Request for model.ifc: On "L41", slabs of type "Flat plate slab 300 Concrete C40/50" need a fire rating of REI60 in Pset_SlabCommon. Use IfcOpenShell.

First a look at what the model holds.

```python
import ifcopenshell
import ifcopenshell.util.element

model = ifcopenshell.open("model.ifc")
print(model.schema)
storey = next(s for s in model.by_type("IfcBuildingStorey") if s.Name == "L41")
slabs = [e for e in ifcopenshell.util.element.get_decomposition(storey) if e.is_a("IfcSlab")]
seen = {}
for e in slabs:
    element_type = ifcopenshell.util.element.get_type(e)
    key = (element_type.Name if element_type != e and element_type else None, ifcopenshell.util.element.get_pset(e, "Pset_SlabCommon", "FireRating"))
    seen[key] = seen.get(key, 0) + 1
for (name, value), count in sorted(seen.items(), key=str):
    print(count, "x", name, "|", value)
```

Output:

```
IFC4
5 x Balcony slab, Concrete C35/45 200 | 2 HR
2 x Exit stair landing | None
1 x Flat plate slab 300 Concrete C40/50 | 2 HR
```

```python
import ifcopenshell
import ifcopenshell.api.pset
import ifcopenshell.util.element

model = ifcopenshell.open("model.ifc")

storey = next(s for s in model.by_type("IfcBuildingStorey") if s.Name == "L41")
slabs = [e for e in ifcopenshell.util.element.get_decomposition(storey) if e.is_a("IfcSlab")]

count = 0
for e in slabs:
    element_type = ifcopenshell.util.element.get_type(e)
    if element_type in (None, e) or element_type.Name != "Flat plate slab 300 Concrete C40/50":
        continue
    found = ifcopenshell.util.element.get_pset(e, "Pset_SlabCommon", should_inherit=False)
    if found:
        pset = model.by_id(found["id"])
        if len(ifcopenshell.util.element.get_elements_by_pset(pset)) > 1:
            pset = ifcopenshell.api.pset.unshare_pset(model, products=[e], pset=pset)[0]
    else:
        pset = ifcopenshell.api.pset.add_pset(model, product=e, name="Pset_SlabCommon")
    ifcopenshell.api.pset.edit_pset(model, pset=pset, properties={"FireRating": "REI60"})
    count += 1

print(count, "slabs updated")

model.write("model_updated.ifc")
```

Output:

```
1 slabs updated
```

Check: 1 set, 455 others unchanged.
